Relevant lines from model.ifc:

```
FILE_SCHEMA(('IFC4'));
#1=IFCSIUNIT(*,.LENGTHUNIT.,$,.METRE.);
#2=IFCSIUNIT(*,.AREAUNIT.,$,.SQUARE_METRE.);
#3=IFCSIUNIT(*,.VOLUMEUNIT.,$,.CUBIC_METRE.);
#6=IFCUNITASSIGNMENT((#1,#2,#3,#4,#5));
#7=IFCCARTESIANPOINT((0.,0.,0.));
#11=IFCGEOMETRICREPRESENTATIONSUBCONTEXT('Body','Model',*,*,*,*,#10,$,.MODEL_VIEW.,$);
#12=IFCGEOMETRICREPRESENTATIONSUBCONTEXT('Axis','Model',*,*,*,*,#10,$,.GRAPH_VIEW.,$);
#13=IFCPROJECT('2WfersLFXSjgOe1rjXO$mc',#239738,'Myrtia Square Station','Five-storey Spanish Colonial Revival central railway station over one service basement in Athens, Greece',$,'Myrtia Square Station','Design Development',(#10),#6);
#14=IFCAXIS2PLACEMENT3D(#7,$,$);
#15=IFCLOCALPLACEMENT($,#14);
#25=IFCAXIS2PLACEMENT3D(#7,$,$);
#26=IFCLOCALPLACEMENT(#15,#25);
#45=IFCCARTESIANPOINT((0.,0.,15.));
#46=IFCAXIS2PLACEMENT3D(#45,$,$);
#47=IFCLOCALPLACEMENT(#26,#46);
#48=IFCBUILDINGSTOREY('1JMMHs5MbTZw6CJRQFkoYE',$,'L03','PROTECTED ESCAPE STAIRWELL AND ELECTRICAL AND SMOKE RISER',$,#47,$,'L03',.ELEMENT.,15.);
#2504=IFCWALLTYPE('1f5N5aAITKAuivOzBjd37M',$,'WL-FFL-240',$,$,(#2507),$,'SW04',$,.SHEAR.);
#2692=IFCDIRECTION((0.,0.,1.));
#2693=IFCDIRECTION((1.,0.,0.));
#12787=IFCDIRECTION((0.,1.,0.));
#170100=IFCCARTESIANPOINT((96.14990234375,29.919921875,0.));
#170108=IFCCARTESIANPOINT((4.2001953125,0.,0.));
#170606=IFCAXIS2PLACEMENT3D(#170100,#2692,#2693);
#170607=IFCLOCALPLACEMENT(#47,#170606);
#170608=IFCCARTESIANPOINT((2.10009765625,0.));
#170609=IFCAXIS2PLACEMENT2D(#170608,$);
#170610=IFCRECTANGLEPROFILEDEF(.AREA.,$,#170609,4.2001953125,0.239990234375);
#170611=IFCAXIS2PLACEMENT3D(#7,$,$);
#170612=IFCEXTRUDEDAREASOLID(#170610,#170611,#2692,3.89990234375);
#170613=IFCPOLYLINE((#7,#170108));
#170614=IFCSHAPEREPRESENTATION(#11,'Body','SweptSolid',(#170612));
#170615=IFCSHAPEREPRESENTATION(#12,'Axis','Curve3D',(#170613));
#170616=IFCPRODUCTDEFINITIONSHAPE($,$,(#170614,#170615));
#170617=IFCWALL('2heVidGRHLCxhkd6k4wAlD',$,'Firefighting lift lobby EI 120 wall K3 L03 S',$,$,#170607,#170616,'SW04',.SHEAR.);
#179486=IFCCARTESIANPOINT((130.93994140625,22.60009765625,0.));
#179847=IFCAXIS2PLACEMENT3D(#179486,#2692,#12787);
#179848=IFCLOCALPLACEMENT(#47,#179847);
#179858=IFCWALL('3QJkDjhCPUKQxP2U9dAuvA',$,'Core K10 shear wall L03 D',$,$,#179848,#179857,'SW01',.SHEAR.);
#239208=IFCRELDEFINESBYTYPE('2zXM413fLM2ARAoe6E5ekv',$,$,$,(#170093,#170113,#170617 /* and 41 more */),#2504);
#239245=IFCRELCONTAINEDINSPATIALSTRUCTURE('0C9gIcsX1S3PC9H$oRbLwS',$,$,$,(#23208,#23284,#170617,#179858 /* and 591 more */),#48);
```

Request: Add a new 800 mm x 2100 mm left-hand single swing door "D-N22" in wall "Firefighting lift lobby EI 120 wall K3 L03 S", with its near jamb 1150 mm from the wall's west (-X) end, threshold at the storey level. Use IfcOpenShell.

```python
import numpy as np
import ifcopenshell
import ifcopenshell.api.feature
import ifcopenshell.api.geometry
import ifcopenshell.api.root
import ifcopenshell.api.spatial
import ifcopenshell.geom
import ifcopenshell.util.element
import ifcopenshell.util.placement
import ifcopenshell.util.representation
import ifcopenshell.util.shape
import ifcopenshell.util.unit

model = ifcopenshell.open("model.ifc")
unit_scale = ifcopenshell.util.unit.calculate_unit_scale(model)
settings = ifcopenshell.geom.settings()


def volume(element):
    """Net volume in cubic metres, openings subtracted."""
    shape = ifcopenshell.geom.create_shape(settings, element)
    return ifcopenshell.util.shape.get_volume(shape.geometry)


wall = model.by_id(170617)
storey = ifcopenshell.util.element.get_container(wall, ifc_class="IfcBuildingStorey")
context = ifcopenshell.util.representation.get_context(model, "Model", "Body", "MODEL_VIEW")
before = volume(wall)

width, height, from_end, sill = 0.8, 2.1, 1.15, 0.0  # metres

# The wall runs along its own X axis, and the end named is its -X end.
wall_shape = ifcopenshell.geom.create_shape(settings, wall)
x, y, z = ifcopenshell.util.shape.get_vertices(wall_shape.geometry).T
start = x.min() + from_end
face, thickness = float(y.min()), float(y.max() - y.min())
wall_matrix = ifcopenshell.util.placement.get_local_placement(wall.ObjectPlacement)
level = ifcopenshell.util.placement.get_local_placement(storey.ObjectPlacement)[2, 3]


def in_wall(x, y):
    """Placement at x, y metres in the wall's axes, at sill height."""
    matrix = wall_matrix.copy()
    matrix[:, 3] = wall_matrix @ np.array([x / unit_scale, y / unit_scale, 0.0, 1.0])
    matrix[2, 3] = level + sill / unit_scale
    return matrix


# Opening: a box that overshoots both wall faces by 50 mm.
opening = ifcopenshell.api.root.create_entity(model, ifc_class="IfcOpeningElement", predefined_type="OPENING")
box = ifcopenshell.api.geometry.add_wall_representation(
    model, context=context, length=width, height=height, thickness=thickness + 0.1
)
ifcopenshell.api.geometry.assign_representation(model, product=opening, representation=box)
ifcopenshell.api.geometry.edit_object_placement(model, product=opening, matrix=in_wall(start, face - 0.05), is_si=False)
ifcopenshell.api.feature.add_feature(model, feature=opening, element=wall)

door = ifcopenshell.api.root.create_entity(model, ifc_class="IfcDoor", name="D-N22", predefined_type="DOOR")
door.OverallWidth, door.OverallHeight = width / unit_scale, height / unit_scale
door.OperationType = "SINGLE_SWING_LEFT"
body = ifcopenshell.api.geometry.add_door_representation(
    model,
    context=context,
    overall_width=door.OverallWidth,
    overall_height=door.OverallHeight,
    operation_type="SINGLE_SWING_LEFT",
    lining_properties={"LiningDepth": thickness / unit_scale, "ThresholdDepth": thickness / unit_scale},
)
ifcopenshell.api.geometry.assign_representation(model, product=door, representation=body)
ifcopenshell.api.spatial.assign_container(model, products=[door], relating_structure=storey)
ifcopenshell.api.feature.add_filling(model, opening=opening, element=door)

# The lining spans the wall, so the door starts at the wall face.
ifcopenshell.api.geometry.edit_object_placement(model, product=door, matrix=in_wall(start, face), is_si=False)

after = volume(wall)

print(f"wall volume {before:.3f} -> {after:.3f} m3")

model.write("model_updated.ifc")
```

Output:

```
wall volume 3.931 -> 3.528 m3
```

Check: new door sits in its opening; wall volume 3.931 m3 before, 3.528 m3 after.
